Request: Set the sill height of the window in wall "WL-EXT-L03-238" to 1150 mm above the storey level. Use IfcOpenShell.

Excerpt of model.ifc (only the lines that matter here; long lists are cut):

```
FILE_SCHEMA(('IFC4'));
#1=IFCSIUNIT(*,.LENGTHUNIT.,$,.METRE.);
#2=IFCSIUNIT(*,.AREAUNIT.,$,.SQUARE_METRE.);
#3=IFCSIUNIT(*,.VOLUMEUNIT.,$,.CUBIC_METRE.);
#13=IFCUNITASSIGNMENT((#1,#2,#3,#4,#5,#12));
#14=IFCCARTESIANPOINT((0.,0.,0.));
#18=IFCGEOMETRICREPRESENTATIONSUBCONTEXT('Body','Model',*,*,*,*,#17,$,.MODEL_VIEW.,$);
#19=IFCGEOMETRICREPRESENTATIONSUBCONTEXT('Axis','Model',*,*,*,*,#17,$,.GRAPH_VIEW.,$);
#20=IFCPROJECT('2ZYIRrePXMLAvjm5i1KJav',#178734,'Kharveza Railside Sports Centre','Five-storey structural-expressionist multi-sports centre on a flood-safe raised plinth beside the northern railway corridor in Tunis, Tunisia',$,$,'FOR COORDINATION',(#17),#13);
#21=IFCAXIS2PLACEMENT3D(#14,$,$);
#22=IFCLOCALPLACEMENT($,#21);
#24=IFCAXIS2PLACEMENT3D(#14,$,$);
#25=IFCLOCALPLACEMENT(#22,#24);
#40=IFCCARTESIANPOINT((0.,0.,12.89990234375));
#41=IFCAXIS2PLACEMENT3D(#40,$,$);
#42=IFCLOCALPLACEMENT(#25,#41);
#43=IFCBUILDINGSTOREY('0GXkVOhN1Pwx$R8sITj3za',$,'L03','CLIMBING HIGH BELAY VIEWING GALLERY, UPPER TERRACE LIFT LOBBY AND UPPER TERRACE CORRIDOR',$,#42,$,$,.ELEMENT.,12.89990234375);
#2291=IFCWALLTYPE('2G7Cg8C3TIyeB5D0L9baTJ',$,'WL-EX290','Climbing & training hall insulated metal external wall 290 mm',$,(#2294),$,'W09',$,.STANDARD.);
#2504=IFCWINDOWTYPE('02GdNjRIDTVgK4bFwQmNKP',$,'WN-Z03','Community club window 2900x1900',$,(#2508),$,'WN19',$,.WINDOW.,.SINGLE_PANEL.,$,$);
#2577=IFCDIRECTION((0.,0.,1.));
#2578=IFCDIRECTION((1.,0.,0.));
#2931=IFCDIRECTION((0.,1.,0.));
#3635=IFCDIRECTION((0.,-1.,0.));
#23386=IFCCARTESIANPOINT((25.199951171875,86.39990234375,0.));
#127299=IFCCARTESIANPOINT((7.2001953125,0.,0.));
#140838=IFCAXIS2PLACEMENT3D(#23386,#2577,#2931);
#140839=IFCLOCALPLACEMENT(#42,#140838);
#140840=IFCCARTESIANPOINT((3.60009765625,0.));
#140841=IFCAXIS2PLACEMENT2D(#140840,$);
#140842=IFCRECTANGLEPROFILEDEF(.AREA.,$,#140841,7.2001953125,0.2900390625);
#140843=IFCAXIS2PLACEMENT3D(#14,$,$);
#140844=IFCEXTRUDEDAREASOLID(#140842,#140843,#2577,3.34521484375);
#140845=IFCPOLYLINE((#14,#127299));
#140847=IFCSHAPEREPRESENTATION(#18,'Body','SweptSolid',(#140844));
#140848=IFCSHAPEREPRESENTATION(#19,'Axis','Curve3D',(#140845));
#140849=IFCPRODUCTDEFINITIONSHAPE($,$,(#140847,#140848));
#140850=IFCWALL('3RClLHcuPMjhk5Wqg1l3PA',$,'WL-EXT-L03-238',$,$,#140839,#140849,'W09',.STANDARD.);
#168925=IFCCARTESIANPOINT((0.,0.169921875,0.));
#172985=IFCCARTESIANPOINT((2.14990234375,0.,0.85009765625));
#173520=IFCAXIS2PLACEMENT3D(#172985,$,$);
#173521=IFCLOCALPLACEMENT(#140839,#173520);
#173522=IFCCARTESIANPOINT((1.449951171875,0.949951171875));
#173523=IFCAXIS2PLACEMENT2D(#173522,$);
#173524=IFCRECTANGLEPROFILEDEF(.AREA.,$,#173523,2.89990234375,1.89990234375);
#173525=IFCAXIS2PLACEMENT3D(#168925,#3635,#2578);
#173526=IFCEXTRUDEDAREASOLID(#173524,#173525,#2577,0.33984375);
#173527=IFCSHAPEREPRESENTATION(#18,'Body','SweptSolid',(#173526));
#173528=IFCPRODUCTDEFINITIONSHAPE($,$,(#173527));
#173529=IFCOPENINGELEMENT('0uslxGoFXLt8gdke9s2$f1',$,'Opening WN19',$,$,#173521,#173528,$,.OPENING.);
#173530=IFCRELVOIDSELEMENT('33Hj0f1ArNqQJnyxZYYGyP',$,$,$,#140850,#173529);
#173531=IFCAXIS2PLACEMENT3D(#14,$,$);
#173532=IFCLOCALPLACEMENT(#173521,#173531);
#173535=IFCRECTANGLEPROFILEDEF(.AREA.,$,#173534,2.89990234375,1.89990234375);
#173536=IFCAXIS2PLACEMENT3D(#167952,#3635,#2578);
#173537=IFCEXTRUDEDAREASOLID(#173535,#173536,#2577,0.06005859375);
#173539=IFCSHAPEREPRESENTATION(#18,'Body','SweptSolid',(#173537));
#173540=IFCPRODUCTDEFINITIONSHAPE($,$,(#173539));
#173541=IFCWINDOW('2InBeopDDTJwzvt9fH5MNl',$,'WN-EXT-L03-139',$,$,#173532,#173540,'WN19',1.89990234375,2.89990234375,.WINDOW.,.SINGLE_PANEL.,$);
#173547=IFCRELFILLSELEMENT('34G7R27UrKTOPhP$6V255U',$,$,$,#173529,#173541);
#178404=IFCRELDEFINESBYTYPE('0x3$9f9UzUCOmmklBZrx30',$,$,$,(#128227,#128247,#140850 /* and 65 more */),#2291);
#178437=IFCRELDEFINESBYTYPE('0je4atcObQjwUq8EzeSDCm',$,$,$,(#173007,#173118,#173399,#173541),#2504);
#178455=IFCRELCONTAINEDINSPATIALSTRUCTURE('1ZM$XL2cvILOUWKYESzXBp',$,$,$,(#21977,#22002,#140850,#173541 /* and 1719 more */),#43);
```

```python
import numpy as np
import ifcopenshell
import ifcopenshell.api.geometry
import ifcopenshell.geom
import ifcopenshell.util.element
import ifcopenshell.util.placement
import ifcopenshell.util.shape
import ifcopenshell.util.unit

model = ifcopenshell.open("model.ifc")
unit_scale = ifcopenshell.util.unit.calculate_unit_scale(model)

window = model.by_guid("2InBeopDDTJwzvt9fH5MNl")
opening = window.FillsVoids[0].RelatingOpeningElement
storey = ifcopenshell.util.element.get_container(window, ifc_class="IfcBuildingStorey")
level = ifcopenshell.util.placement.get_local_placement(storey.ObjectPlacement)[2, 3]

# The opening's origin need not be at the sill, so measure its lowest point.
shape = ifcopenshell.geom.create_shape(ifcopenshell.geom.settings(), opening)
bottom = ifcopenshell.util.shape.get_shape_bottom_elevation(shape, shape.geometry) / unit_scale
dz = level + 1.15 / unit_scale - bottom

shift = np.array([0.0, 0.0, dz])
# The window is placed relative to its opening, so it follows when the opening moves.
matrix = ifcopenshell.util.placement.get_local_placement(opening.ObjectPlacement)
matrix[:3, 3] += shift
ifcopenshell.api.geometry.edit_object_placement(
    model, product=opening, matrix=matrix, is_si=False, should_transform_children=True
)

print(f"moved by {dz * unit_scale:+.3f} m")

model.write("model_edited.ifc")
```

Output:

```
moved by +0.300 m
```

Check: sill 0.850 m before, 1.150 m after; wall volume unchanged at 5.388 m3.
